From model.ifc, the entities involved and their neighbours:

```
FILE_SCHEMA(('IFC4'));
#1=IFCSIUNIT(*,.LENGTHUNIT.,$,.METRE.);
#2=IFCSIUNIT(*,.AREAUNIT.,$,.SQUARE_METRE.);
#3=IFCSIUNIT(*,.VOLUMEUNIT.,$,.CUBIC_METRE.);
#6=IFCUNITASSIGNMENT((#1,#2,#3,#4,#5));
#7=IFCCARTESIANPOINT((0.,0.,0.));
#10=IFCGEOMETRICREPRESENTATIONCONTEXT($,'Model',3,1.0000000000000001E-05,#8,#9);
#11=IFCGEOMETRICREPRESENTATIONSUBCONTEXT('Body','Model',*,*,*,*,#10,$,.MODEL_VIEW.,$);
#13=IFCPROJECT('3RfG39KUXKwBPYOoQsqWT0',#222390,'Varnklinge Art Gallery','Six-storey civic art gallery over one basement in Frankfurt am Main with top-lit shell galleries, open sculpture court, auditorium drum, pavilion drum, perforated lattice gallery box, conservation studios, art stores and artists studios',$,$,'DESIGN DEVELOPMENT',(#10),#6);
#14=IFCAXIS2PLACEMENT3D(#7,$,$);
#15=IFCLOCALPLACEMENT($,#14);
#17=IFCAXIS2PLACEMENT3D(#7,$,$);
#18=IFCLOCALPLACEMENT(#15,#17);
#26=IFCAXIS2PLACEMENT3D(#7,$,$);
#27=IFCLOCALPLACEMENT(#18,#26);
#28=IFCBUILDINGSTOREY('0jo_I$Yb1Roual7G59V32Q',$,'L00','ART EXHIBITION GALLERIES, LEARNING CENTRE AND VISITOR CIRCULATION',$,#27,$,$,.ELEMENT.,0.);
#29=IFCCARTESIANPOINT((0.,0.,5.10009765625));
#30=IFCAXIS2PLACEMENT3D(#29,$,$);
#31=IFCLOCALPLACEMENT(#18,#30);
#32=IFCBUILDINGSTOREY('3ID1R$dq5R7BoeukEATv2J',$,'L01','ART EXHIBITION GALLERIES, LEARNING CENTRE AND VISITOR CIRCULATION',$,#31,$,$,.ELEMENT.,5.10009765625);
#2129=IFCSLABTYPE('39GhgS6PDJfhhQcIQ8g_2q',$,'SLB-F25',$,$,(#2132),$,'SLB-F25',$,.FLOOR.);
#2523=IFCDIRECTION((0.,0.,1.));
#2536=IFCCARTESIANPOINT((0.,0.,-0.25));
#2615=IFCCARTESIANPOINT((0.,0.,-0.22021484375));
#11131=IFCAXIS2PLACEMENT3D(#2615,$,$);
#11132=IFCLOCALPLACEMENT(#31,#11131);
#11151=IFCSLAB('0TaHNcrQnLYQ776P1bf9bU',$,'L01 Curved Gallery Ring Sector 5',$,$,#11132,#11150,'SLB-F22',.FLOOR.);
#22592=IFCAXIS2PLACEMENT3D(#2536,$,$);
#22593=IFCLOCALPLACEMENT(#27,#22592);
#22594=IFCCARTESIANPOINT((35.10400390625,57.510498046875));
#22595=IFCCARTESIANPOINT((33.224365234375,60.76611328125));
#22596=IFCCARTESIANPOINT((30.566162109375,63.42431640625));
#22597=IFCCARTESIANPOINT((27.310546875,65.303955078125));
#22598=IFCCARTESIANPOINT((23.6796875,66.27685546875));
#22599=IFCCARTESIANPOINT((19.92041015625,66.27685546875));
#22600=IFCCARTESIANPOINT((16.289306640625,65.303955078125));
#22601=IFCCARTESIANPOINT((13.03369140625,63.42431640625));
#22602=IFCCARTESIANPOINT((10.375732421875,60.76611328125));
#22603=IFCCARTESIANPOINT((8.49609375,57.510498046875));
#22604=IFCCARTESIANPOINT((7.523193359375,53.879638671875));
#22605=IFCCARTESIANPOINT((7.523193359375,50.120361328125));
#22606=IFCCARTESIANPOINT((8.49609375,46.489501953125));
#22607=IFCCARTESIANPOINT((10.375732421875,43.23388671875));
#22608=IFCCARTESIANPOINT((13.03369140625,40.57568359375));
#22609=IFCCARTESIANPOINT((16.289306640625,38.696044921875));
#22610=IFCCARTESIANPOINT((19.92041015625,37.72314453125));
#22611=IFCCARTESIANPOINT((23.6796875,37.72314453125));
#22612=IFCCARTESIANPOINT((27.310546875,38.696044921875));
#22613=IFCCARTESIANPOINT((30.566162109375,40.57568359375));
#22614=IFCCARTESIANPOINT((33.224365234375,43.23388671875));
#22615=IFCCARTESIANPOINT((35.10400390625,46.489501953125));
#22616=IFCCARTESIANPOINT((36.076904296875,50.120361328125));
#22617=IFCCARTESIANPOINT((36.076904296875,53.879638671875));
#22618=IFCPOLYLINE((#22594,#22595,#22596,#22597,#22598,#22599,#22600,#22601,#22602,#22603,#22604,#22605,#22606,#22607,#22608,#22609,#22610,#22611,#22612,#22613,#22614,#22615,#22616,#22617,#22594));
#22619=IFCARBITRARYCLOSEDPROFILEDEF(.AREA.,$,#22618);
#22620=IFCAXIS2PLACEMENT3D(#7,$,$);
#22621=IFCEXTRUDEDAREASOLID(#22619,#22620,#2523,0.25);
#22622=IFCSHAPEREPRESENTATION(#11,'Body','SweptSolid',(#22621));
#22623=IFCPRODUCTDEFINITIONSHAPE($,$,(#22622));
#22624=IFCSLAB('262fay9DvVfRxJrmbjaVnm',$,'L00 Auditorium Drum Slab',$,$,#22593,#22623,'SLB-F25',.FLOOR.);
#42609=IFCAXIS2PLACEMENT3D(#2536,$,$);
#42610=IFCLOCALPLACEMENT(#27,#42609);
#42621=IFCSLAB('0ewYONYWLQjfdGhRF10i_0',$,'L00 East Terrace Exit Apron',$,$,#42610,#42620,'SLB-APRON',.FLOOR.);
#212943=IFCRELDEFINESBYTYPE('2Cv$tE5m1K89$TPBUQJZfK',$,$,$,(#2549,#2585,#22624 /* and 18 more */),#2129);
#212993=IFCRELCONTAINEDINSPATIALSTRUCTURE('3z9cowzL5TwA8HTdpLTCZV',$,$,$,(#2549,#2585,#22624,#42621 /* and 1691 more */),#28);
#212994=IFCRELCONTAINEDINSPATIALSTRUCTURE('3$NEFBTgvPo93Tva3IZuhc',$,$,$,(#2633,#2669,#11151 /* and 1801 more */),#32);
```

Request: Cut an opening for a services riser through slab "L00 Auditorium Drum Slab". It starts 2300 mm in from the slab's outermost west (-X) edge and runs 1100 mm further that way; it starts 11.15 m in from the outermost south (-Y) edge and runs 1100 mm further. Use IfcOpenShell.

```python
import numpy as np
import ifcopenshell
import ifcopenshell.api.feature
import ifcopenshell.api.geometry
import ifcopenshell.api.root
import ifcopenshell.geom
import ifcopenshell.util.placement
import ifcopenshell.util.representation
import ifcopenshell.util.shape
import ifcopenshell.util.unit

model = ifcopenshell.open("model.ifc")
unit_scale = ifcopenshell.util.unit.calculate_unit_scale(model)
settings = ifcopenshell.geom.settings()


def volume(element):
    """Net volume in cubic metres, openings subtracted."""
    shape = ifcopenshell.geom.create_shape(settings, element)
    return ifcopenshell.util.shape.get_volume(shape.geometry)


slab = model.by_id(22624)
before = volume(slab)

# Extent in the slab's own axes, in metres. The edges named are its -X and -Y sides.
slab_shape = ifcopenshell.geom.create_shape(settings, slab)
vertices = ifcopenshell.util.shape.get_vertices(slab_shape.geometry)
x_min, y_min, bottom = vertices.min(axis=0)
top = vertices[:, 2].max()

opening = ifcopenshell.api.root.create_entity(model, ifc_class="IfcOpeningElement", name="Services riser opening", predefined_type="OPENING")
context = ifcopenshell.util.representation.get_context(model, "Model", "Body", "MODEL_VIEW")
width, depth = 1.1, 1.1
outline = [(0.0, 0.0), (width, 0.0), (width, depth), (0.0, depth), (0.0, 0.0)]
# Overshoot both faces by 50 mm so the cut is clean.
shape = ifcopenshell.api.geometry.add_slab_representation(
    model, context=context, depth=top - bottom + 0.1, polyline=outline
)
ifcopenshell.api.geometry.assign_representation(model, product=opening, representation=shape)

matrix = ifcopenshell.util.placement.get_local_placement(slab.ObjectPlacement)
matrix[:, 3] = matrix @ np.append(np.array([x_min + 2.3, y_min + 11.15, bottom - 0.05]) / unit_scale, 1.0)
ifcopenshell.api.geometry.edit_object_placement(model, product=opening, matrix=matrix, is_si=False)
ifcopenshell.api.feature.add_feature(model, feature=opening, element=slab)

after = volume(slab)

print(f"slab volume {before:.3f} -> {after:.3f} m3")

model.write("model_rev.ifc")
```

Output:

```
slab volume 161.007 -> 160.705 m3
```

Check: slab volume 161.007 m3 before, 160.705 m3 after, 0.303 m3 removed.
